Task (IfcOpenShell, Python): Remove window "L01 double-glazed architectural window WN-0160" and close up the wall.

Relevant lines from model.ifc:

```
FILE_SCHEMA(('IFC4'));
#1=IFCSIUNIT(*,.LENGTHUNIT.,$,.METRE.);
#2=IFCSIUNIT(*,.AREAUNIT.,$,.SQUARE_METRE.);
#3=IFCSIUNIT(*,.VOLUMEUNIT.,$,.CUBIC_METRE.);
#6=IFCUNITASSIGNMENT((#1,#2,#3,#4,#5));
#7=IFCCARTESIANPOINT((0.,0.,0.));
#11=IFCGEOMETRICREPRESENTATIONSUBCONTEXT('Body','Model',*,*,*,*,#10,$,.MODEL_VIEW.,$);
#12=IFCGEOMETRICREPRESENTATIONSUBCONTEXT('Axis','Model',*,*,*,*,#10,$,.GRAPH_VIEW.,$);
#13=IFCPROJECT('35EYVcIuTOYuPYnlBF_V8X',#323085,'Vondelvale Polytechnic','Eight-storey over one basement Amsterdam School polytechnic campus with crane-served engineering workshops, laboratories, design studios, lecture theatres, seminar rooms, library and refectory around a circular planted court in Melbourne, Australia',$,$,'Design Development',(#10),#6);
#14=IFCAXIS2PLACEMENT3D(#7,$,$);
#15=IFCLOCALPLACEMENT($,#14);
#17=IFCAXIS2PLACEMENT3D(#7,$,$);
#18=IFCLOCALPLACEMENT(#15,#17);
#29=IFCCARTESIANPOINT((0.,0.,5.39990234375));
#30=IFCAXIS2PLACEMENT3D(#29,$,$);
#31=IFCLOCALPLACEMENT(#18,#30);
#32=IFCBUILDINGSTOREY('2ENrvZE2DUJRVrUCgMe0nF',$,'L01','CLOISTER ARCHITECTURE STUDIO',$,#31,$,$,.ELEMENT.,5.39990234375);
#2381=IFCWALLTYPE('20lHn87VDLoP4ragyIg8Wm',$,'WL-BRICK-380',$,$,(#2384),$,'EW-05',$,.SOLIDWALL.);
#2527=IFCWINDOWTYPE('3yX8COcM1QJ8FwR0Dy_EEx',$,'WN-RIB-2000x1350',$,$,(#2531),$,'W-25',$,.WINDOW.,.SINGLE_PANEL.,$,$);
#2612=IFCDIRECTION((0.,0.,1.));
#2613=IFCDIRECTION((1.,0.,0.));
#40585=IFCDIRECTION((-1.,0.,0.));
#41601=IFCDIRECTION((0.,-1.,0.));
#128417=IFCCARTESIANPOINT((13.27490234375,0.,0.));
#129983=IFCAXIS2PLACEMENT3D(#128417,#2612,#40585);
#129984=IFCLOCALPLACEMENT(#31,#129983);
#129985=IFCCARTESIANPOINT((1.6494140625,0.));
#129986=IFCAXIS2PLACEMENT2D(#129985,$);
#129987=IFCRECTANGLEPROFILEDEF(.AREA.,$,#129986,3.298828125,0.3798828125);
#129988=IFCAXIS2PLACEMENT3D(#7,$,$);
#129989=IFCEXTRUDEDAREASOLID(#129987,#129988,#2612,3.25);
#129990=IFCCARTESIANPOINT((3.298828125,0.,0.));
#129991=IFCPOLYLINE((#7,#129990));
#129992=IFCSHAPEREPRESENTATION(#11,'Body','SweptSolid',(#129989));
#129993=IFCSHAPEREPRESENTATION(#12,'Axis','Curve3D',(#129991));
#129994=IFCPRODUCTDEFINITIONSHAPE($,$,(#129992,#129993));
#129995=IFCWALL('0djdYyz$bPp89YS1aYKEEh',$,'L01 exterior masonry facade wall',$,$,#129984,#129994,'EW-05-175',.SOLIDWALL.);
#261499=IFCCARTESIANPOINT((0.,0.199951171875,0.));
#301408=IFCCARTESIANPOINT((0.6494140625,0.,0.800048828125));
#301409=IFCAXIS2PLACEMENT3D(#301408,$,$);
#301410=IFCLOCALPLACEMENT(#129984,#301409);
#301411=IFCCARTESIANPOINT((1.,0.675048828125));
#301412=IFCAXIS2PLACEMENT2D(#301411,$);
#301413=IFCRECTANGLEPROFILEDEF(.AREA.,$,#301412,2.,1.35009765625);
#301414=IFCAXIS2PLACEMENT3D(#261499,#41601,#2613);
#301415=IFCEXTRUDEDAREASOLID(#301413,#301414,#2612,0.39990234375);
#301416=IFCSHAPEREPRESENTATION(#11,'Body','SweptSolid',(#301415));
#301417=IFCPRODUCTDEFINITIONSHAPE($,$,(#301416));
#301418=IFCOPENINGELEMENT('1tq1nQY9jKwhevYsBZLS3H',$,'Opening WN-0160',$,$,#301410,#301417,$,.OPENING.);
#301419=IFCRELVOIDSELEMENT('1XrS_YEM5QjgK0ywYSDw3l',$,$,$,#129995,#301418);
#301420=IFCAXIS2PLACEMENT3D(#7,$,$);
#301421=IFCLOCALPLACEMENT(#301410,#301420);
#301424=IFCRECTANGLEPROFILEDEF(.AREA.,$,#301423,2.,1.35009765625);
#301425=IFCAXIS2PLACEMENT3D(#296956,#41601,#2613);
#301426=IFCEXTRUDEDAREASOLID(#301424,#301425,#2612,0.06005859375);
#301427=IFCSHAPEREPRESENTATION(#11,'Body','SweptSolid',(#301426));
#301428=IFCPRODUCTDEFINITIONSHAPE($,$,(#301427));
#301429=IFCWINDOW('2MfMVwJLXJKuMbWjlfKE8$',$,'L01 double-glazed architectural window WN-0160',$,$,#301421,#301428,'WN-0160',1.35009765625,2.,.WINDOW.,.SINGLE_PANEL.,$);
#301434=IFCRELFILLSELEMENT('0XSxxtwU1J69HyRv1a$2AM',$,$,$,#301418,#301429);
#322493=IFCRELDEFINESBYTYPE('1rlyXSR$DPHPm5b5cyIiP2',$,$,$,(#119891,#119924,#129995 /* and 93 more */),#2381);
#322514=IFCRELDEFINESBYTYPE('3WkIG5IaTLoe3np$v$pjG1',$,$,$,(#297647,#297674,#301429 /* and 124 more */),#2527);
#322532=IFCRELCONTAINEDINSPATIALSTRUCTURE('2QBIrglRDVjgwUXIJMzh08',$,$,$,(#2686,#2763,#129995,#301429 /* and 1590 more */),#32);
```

```python
import ifcopenshell
import ifcopenshell.api.feature
import ifcopenshell.api.root
import ifcopenshell.geom
import ifcopenshell.util.shape

model = ifcopenshell.open("model.ifc")
settings = ifcopenshell.geom.settings()


def volume(element):
    """Net volume in cubic metres, openings subtracted."""
    shape = ifcopenshell.geom.create_shape(settings, element)
    return ifcopenshell.util.shape.get_volume(shape.geometry)


window = model.by_guid("2MfMVwJLXJKuMbWjlfKE8$")
opening = window.FillsVoids[0].RelatingOpeningElement
wall = opening.VoidsElements[0].RelatingBuildingElement
before = volume(wall)

ifcopenshell.api.root.remove_product(model, product=window)
ifcopenshell.api.feature.remove_feature(model, feature=opening)

after = volume(wall)

print(f"wall volume {before:.3f} -> {after:.3f} m3")

model.write("model_updated.ifc")
```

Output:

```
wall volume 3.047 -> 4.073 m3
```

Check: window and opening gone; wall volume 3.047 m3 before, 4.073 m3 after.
